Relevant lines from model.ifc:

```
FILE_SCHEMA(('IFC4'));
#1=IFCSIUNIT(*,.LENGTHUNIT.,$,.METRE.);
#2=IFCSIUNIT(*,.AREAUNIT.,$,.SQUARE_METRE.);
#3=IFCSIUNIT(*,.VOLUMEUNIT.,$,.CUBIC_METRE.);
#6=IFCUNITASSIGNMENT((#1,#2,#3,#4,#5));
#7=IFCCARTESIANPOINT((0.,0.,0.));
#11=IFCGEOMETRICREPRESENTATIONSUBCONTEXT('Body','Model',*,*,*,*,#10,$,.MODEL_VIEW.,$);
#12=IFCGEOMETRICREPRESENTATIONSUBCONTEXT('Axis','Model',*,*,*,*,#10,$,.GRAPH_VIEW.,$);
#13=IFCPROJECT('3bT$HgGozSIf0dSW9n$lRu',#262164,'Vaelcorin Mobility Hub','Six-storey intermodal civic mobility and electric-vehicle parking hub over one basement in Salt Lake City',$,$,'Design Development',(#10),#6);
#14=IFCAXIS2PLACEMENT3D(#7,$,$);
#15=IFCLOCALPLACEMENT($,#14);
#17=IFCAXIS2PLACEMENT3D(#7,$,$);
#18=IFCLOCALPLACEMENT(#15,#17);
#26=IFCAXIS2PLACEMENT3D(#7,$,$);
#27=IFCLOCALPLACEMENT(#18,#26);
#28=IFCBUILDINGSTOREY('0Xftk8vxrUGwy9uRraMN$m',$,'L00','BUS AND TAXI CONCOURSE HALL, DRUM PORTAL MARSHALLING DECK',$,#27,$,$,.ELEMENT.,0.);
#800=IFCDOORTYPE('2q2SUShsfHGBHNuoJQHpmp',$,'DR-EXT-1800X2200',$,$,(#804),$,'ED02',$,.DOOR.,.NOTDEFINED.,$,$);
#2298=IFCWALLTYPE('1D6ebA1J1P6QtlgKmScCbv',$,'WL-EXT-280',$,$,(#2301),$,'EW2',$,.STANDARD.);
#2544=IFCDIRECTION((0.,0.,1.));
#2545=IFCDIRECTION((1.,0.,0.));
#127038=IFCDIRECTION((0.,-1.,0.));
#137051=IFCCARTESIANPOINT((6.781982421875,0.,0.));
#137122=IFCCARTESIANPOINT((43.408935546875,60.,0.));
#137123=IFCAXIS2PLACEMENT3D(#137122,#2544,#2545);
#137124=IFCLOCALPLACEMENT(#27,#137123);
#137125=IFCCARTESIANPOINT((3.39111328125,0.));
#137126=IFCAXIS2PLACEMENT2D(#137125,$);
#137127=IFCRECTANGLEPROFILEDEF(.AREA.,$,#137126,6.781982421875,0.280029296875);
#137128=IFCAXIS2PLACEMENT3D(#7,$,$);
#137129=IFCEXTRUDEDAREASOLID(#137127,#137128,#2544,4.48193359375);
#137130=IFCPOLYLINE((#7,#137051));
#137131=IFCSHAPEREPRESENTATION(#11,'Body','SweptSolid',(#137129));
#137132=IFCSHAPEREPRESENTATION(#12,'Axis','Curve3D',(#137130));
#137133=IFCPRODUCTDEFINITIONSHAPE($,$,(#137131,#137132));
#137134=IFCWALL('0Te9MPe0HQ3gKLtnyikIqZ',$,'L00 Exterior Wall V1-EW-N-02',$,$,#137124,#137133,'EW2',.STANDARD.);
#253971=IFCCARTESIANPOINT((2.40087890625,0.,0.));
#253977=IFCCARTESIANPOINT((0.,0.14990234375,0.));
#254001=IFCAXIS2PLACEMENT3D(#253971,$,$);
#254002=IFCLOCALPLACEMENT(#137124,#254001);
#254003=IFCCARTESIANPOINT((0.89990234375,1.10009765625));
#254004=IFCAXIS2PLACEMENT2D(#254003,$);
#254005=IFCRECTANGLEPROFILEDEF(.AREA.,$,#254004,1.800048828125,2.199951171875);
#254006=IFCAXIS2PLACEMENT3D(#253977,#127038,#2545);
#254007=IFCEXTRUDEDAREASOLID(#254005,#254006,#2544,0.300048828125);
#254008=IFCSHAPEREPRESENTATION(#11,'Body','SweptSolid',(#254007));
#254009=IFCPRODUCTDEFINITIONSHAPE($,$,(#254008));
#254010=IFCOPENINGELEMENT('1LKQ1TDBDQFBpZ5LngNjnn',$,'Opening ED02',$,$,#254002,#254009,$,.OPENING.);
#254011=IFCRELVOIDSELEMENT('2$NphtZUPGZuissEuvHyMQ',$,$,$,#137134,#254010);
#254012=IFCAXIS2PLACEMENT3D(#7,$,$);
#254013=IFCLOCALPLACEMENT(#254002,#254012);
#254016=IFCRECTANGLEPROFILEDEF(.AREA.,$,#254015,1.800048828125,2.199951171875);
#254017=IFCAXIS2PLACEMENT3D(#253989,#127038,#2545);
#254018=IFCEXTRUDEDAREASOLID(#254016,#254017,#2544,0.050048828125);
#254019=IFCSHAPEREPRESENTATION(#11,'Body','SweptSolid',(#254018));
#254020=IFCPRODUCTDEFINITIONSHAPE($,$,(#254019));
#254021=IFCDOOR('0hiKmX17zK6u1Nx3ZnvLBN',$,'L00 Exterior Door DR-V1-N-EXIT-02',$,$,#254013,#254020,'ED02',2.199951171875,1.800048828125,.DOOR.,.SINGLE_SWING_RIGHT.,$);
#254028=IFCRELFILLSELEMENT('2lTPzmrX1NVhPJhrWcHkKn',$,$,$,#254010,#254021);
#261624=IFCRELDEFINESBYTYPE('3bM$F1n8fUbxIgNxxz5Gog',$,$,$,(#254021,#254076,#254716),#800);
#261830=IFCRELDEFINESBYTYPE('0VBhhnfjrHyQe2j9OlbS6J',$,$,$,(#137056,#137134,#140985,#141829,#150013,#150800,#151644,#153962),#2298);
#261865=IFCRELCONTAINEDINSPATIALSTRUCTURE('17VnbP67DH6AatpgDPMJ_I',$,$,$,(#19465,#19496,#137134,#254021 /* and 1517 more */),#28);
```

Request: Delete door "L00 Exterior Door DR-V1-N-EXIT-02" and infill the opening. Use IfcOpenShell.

```python
import ifcopenshell
import ifcopenshell.api.feature
import ifcopenshell.api.root
import ifcopenshell.geom
import ifcopenshell.util.shape

model = ifcopenshell.open("model.ifc")
settings = ifcopenshell.geom.settings()


def volume(element):
    """Net volume in cubic metres, openings subtracted."""
    shape = ifcopenshell.geom.create_shape(settings, element)
    return ifcopenshell.util.shape.get_volume(shape.geometry)


door = model.by_guid("0hiKmX17zK6u1Nx3ZnvLBN")
opening = door.FillsVoids[0].RelatingOpeningElement
wall = opening.VoidsElements[0].RelatingBuildingElement
before = volume(wall)

ifcopenshell.api.root.remove_product(model, product=door)
ifcopenshell.api.feature.remove_feature(model, feature=opening)

after = volume(wall)

print(f"wall volume {before:.3f} -> {after:.3f} m3")

model.write("model-out.ifc")
```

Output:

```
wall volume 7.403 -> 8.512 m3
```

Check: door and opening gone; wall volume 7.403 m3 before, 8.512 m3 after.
